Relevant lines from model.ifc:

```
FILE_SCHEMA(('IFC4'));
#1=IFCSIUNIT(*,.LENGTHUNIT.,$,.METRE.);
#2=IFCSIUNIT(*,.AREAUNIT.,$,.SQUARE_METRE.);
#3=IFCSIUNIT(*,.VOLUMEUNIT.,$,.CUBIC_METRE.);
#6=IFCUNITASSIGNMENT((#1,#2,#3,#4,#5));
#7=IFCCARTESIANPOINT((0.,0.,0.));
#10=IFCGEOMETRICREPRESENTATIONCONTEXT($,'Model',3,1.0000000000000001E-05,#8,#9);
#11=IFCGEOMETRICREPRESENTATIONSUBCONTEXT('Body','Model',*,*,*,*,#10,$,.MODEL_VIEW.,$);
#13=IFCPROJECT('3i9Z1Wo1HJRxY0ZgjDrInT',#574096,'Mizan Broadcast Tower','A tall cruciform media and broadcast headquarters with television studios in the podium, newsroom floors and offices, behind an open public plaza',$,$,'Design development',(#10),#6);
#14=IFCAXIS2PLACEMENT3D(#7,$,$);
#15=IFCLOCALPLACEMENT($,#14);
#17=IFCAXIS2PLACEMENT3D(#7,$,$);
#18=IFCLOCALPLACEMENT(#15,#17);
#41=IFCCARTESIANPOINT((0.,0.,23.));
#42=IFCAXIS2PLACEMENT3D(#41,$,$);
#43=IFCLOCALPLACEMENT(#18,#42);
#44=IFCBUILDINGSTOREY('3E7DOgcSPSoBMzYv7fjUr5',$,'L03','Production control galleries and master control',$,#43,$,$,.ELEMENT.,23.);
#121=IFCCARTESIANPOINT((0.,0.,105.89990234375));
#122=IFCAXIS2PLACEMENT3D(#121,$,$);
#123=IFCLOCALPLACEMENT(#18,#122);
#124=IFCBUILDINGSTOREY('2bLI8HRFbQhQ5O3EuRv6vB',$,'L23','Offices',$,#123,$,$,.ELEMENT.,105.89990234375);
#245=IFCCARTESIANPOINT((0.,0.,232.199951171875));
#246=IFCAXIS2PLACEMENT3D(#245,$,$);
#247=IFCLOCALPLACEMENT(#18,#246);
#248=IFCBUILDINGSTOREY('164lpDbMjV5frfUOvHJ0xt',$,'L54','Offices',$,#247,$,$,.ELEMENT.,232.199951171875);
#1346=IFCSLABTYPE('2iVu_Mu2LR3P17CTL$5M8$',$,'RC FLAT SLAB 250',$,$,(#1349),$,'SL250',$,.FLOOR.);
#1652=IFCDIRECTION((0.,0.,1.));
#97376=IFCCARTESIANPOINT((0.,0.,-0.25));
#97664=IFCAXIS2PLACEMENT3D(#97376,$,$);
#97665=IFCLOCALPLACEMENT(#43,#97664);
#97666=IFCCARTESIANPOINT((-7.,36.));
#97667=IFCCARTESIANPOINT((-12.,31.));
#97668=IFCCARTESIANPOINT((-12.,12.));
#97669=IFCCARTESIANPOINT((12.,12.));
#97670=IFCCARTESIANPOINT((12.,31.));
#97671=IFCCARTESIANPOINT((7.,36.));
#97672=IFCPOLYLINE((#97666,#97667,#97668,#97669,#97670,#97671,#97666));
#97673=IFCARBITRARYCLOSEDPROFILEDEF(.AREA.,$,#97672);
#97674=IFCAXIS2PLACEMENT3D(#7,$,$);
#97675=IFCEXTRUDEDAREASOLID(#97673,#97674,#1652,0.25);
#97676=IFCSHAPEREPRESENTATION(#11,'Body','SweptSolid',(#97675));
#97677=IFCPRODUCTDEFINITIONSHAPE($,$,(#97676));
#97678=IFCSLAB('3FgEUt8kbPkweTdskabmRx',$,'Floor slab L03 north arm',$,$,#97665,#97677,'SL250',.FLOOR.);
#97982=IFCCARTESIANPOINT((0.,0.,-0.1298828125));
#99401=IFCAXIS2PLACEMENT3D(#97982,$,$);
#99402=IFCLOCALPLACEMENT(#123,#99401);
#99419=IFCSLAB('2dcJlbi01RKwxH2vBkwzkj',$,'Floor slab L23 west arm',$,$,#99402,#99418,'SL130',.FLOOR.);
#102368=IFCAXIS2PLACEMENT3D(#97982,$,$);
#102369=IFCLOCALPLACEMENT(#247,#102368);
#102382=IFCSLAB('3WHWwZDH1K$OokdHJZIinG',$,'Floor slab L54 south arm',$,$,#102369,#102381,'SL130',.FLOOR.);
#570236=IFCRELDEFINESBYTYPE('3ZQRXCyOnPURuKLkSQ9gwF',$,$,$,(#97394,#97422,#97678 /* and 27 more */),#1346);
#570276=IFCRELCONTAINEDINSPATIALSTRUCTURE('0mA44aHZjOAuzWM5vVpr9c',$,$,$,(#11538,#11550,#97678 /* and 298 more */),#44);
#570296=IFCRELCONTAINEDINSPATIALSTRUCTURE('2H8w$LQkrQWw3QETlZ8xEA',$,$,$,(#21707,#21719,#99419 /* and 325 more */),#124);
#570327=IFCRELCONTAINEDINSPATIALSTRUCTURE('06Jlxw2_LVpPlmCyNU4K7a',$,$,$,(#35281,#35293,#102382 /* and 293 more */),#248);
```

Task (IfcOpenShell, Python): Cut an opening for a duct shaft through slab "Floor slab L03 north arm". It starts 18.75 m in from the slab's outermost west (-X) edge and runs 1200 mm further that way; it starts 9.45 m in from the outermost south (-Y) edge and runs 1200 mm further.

```python
import numpy as np
import ifcopenshell
import ifcopenshell.api.feature
import ifcopenshell.api.geometry
import ifcopenshell.api.root
import ifcopenshell.geom
import ifcopenshell.util.placement
import ifcopenshell.util.representation
import ifcopenshell.util.shape
import ifcopenshell.util.unit

model = ifcopenshell.open("model.ifc")
unit_scale = ifcopenshell.util.unit.calculate_unit_scale(model)
settings = ifcopenshell.geom.settings()


def volume(element):
    """Net volume in cubic metres, openings subtracted."""
    shape = ifcopenshell.geom.create_shape(settings, element)
    return ifcopenshell.util.shape.get_volume(shape.geometry)


slab = model.by_id(97678)
before = volume(slab)

# Extent in the slab's own axes, in metres. The edges named are its -X and -Y sides.
slab_shape = ifcopenshell.geom.create_shape(settings, slab)
vertices = ifcopenshell.util.shape.get_vertices(slab_shape.geometry)
x_min, y_min, bottom = vertices.min(axis=0)
top = vertices[:, 2].max()

opening = ifcopenshell.api.root.create_entity(model, ifc_class="IfcOpeningElement", name="Duct shaft opening", predefined_type="OPENING")
context = ifcopenshell.util.representation.get_context(model, "Model", "Body", "MODEL_VIEW")
width, depth = 1.2, 1.2
outline = [(0.0, 0.0), (width, 0.0), (width, depth), (0.0, depth), (0.0, 0.0)]
# Overshoot both faces by 50 mm so the cut is clean.
shape = ifcopenshell.api.geometry.add_slab_representation(
    model, context=context, depth=top - bottom + 0.1, polyline=outline
)
ifcopenshell.api.geometry.assign_representation(model, product=opening, representation=shape)

matrix = ifcopenshell.util.placement.get_local_placement(slab.ObjectPlacement)
matrix[:, 3] = matrix @ np.append(np.array([x_min + 18.75, y_min + 9.45, bottom - 0.05]) / unit_scale, 1.0)
ifcopenshell.api.geometry.edit_object_placement(model, product=opening, matrix=matrix, is_si=False)
ifcopenshell.api.feature.add_feature(model, feature=opening, element=slab)

after = volume(slab)

print(f"slab volume {before:.3f} -> {after:.3f} m3")

model.write("model_v2.ifc")
```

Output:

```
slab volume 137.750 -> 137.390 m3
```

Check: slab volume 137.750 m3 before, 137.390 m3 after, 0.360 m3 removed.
